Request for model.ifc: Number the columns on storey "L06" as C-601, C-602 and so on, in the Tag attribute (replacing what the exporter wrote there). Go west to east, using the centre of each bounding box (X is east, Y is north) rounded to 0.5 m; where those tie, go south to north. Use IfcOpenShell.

First a look at what the model holds.

```python
import ifcopenshell
import ifcopenshell.util.element
import ifcopenshell.util.placement

model = ifcopenshell.open("model.ifc")
print(model.schema)
storey = next(s for s in model.by_type("IfcBuildingStorey") if s.Name == "L06")
columns = [e for e in ifcopenshell.util.element.get_decomposition(storey) if e.is_a("IfcColumn")]
for e in sorted(columns, key=lambda e: e.id()):
    origin = ifcopenshell.util.placement.get_local_placement(e.ObjectPlacement)[:3, 3]
    print(e.id(), e.Tag, e.Name, origin.round(2) + 0.0, sep=" | ")
```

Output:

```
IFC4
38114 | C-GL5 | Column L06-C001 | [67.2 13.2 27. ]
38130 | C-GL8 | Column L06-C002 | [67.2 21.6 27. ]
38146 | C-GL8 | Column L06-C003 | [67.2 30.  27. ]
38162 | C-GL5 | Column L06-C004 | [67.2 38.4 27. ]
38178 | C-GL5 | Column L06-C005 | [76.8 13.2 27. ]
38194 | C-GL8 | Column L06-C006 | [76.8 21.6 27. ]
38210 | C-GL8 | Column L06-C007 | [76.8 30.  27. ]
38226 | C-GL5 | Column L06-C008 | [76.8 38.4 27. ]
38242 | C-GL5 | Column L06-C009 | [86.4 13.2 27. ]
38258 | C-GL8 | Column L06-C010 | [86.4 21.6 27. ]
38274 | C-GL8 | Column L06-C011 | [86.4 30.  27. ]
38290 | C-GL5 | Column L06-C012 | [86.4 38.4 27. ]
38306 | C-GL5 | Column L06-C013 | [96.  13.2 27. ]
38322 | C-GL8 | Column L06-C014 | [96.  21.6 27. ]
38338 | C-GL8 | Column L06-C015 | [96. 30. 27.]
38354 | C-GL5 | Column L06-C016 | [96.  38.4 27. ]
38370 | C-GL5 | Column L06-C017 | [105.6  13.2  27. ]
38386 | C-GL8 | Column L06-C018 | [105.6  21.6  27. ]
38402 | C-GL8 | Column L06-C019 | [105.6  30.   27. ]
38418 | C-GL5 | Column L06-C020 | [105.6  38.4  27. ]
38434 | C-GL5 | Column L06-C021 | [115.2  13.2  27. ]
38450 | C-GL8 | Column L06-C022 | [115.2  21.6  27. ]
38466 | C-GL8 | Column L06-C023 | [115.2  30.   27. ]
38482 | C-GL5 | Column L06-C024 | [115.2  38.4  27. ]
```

```python
import ifcopenshell
import ifcopenshell.geom
import ifcopenshell.util.element
import ifcopenshell.util.shape

model = ifcopenshell.open("model.ifc")
settings = ifcopenshell.geom.settings()
settings.set("use-world-coords", True)


def centre(element):
    shape = ifcopenshell.geom.create_shape(settings, element)
    return ifcopenshell.util.shape.get_bbox_centroid(shape.geometry)


storey = next(s for s in model.by_type("IfcBuildingStorey") if s.Name == "L06")
columns = [e for e in ifcopenshell.util.element.get_decomposition(storey) if e.is_a("IfcColumn")]

# Insertion points can sit at a corner or the storey origin, so sort by the geometry (in metres).
centres = {e: centre(e) for e in columns}
columns.sort(key=lambda e: (round(centres[e][0] / 0.5), centres[e][1]))

for i, e in enumerate(columns, start=1):
    number = f"C-6{i:02d}"
    e.Tag = number
    print(e.id(), number)

model.write("model_edited.ifc")
```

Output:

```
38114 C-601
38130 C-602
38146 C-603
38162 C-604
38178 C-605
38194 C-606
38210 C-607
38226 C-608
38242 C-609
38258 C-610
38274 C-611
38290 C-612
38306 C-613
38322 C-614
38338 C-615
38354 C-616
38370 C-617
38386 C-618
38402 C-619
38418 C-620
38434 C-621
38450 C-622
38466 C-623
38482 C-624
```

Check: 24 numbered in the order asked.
